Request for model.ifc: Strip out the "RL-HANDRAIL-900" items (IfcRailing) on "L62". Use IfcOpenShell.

First a look at what the model holds.

```python
import ifcopenshell
import ifcopenshell.util.element

model = ifcopenshell.open("model.ifc")
print(model.schema)
storey = next(s for s in model.by_type("IfcBuildingStorey") if s.Name == "L62")
railings = [e for e in ifcopenshell.util.element.get_decomposition(storey) if e.is_a("IfcRailing")]
seen = {}
for e in railings:
    element_type = ifcopenshell.util.element.get_type(e)
    name = element_type.Name if element_type not in (None, e) else None
    seen[name] = seen.get(name, 0) + 1
for name, count in sorted(seen.items(), key=str):
    print(count, "x", name)
```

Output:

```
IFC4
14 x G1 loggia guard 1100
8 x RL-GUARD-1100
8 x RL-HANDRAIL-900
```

```python
import ifcopenshell
import ifcopenshell.api.root
import ifcopenshell.util.element

model = ifcopenshell.open("model.ifc")

storey = next(s for s in model.by_type("IfcBuildingStorey") if s.Name == "L62")
railings = [e for e in ifcopenshell.util.element.get_decomposition(storey) if e.is_a("IfcRailing")]
targets = [e for e in railings if (t := ifcopenshell.util.element.get_type(e)) not in (None, e) and t.Name == "RL-HANDRAIL-900"]

for e in targets:
    ifcopenshell.api.root.remove_product(model, product=e)
print(len(targets), "removed")

model.write("model-out.ifc")
```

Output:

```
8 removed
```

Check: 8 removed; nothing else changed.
